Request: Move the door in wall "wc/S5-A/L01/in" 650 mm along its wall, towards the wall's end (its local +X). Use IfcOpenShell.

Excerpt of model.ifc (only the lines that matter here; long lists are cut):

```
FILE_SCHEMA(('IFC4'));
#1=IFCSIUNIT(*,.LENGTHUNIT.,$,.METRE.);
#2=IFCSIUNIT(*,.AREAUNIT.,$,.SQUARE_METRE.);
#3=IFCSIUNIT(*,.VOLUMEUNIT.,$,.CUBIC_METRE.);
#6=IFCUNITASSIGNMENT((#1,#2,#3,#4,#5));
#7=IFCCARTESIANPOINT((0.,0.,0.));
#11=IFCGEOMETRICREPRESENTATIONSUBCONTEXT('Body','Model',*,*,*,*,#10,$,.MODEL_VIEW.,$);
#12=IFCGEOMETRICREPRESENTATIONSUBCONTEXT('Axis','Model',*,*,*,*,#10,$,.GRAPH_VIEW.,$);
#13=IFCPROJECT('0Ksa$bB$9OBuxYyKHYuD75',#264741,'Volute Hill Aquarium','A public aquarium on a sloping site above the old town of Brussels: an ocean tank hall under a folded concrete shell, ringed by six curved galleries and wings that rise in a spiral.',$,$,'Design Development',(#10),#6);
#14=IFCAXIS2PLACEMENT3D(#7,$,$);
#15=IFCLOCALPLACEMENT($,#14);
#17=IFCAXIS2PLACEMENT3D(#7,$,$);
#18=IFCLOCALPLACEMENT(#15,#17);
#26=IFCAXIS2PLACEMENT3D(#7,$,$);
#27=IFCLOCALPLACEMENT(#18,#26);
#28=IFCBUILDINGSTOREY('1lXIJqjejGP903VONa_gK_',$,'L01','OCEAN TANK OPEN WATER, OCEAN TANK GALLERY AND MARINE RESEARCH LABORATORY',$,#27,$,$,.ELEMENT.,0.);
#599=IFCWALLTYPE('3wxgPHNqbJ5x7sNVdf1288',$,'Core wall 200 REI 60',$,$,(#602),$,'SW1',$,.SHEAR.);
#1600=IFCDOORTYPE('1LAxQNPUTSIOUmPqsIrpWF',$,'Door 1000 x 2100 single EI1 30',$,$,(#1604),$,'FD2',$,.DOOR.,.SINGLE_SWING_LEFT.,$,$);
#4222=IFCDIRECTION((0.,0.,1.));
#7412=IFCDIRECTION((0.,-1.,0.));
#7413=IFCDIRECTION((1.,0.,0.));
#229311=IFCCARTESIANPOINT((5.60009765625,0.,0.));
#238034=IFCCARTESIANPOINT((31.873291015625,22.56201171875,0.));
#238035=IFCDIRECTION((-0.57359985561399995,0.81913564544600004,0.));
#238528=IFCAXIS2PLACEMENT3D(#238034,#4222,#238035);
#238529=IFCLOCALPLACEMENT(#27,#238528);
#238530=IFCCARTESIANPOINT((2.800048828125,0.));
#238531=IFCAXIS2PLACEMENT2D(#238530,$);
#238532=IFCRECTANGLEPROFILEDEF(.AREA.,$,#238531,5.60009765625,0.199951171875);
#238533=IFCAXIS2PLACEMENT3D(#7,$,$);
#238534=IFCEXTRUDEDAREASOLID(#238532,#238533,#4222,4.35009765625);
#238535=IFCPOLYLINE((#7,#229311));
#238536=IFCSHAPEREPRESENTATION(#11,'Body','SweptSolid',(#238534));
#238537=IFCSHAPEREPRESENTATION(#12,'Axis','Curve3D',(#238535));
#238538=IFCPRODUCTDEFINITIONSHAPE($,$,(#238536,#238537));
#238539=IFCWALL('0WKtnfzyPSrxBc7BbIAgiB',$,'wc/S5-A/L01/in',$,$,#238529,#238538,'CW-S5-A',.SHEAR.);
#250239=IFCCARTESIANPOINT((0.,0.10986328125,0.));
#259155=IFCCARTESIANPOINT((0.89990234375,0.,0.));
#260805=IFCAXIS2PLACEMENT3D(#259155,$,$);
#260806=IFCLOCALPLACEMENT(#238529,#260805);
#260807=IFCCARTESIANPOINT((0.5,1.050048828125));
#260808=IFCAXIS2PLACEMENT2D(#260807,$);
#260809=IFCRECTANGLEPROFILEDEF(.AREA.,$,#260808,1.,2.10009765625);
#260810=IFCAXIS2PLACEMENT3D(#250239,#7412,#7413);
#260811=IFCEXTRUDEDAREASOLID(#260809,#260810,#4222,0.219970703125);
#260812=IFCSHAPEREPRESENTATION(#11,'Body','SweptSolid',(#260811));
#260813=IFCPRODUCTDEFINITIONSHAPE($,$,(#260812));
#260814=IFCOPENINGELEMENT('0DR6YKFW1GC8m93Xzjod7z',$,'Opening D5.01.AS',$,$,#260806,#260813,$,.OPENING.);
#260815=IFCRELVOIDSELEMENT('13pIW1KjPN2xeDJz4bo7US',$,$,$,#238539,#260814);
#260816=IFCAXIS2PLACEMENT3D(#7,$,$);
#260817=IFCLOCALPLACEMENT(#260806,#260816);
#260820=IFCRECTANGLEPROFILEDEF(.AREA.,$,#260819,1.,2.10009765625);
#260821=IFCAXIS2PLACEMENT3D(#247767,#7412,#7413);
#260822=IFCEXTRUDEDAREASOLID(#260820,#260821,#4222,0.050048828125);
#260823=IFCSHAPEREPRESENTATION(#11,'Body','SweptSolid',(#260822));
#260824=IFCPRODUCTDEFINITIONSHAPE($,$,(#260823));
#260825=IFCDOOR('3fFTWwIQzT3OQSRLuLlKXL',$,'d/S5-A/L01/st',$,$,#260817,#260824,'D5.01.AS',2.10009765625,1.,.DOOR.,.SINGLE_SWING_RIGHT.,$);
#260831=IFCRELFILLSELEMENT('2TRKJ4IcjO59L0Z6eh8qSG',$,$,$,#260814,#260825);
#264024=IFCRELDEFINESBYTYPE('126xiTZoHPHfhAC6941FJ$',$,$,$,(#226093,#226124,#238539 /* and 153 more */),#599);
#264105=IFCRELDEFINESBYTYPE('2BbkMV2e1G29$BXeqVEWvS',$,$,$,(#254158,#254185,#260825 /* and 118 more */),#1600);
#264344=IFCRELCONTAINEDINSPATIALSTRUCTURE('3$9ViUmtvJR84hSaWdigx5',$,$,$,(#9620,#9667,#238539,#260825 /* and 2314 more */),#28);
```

```python
import ifcopenshell
import ifcopenshell.api.geometry
import ifcopenshell.util.placement
import ifcopenshell.util.unit

model = ifcopenshell.open("model.ifc")
unit_scale = ifcopenshell.util.unit.calculate_unit_scale(model)

door = model.by_guid("3fFTWwIQzT3OQSRLuLlKXL")
opening = door.FillsVoids[0].RelatingOpeningElement
wall = opening.VoidsElements[0].RelatingBuildingElement

wall_matrix = ifcopenshell.util.placement.get_local_placement(wall.ObjectPlacement)
shift = wall_matrix[:3, 0] * 0.65 / unit_scale
before = ifcopenshell.util.placement.get_local_placement(door.ObjectPlacement)[:3, 3].copy()

# The door is placed relative to its opening, so it follows when the opening moves.
matrix = ifcopenshell.util.placement.get_local_placement(opening.ObjectPlacement)
matrix[:3, 3] += shift
ifcopenshell.api.geometry.edit_object_placement(
    model, product=opening, matrix=matrix, is_si=False, should_transform_children=True
)

after = ifcopenshell.util.placement.get_local_placement(door.ObjectPlacement)[:3, 3]
print("door moved by", (after - before).round(3) + 0.0)

model.write("model-out.ifc")
```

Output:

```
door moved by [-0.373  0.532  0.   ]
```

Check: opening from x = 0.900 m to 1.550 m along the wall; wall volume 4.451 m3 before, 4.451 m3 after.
